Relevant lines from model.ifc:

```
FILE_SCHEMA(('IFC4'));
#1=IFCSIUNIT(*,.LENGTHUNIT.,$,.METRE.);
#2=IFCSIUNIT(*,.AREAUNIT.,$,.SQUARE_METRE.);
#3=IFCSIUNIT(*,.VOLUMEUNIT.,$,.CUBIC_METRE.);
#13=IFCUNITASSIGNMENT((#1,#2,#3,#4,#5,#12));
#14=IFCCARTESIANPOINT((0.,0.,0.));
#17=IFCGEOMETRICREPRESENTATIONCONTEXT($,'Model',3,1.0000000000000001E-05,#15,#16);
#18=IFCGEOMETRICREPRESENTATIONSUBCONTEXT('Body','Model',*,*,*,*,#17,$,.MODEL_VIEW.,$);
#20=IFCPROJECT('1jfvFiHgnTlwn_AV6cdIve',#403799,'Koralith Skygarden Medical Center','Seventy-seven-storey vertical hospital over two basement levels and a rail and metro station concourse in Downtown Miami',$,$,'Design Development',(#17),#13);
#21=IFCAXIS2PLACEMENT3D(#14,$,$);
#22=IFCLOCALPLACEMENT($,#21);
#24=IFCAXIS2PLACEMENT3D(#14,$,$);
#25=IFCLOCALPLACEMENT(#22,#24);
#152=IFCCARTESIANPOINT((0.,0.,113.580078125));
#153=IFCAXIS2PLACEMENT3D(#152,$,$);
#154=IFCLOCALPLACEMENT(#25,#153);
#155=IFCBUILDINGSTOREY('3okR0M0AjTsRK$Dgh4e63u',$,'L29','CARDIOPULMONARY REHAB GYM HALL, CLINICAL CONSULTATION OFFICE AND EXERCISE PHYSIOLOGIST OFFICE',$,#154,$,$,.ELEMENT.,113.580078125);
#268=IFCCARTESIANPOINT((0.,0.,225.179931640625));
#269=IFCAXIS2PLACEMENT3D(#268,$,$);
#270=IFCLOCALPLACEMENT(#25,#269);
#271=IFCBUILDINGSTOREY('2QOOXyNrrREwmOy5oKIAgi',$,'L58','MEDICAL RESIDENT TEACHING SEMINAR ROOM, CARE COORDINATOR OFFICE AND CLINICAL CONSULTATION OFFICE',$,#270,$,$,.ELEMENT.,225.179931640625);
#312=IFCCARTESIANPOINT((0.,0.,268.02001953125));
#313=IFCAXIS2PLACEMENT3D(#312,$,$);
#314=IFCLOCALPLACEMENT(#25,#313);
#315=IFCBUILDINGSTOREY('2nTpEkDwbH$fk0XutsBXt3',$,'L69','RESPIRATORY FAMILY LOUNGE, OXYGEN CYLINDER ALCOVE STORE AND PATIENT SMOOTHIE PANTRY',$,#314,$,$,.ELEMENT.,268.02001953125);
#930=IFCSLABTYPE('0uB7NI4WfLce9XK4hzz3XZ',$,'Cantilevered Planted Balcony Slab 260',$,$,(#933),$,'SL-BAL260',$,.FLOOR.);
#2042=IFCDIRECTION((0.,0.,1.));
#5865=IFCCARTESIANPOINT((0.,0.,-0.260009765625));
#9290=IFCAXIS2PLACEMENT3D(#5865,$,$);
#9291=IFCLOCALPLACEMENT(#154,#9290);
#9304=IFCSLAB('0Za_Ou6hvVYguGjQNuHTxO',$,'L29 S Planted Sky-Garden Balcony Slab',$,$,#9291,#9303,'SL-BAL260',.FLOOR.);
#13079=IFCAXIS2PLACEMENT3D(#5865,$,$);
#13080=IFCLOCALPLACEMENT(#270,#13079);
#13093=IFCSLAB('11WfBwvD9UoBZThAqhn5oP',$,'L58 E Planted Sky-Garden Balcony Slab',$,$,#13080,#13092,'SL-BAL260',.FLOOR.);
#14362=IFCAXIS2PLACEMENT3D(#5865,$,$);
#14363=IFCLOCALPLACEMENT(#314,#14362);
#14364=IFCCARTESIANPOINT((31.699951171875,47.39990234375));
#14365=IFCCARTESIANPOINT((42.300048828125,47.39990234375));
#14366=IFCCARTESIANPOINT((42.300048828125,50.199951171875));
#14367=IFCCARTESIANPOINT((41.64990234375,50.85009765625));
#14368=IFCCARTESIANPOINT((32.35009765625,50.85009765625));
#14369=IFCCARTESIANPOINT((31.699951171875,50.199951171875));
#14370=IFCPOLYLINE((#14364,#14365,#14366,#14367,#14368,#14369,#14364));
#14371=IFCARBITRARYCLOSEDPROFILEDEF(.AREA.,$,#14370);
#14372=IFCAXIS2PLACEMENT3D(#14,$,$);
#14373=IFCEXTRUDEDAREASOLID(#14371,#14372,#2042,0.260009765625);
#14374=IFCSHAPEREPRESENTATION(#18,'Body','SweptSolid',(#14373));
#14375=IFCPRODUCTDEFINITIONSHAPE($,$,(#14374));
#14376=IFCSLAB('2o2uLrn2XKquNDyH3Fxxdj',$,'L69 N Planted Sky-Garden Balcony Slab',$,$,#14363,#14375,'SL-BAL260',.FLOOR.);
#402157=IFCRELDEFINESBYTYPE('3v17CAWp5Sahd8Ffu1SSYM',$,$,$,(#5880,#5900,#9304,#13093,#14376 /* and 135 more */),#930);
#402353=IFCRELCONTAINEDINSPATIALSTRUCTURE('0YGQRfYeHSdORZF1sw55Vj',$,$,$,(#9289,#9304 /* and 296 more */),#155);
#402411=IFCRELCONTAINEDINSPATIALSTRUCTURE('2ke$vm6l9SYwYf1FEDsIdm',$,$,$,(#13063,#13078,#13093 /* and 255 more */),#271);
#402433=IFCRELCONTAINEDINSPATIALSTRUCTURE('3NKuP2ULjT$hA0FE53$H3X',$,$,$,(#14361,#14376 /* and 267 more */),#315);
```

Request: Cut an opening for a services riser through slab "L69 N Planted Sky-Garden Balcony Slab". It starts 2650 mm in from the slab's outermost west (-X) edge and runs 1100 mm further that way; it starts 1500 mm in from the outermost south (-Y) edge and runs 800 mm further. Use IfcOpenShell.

```python
import numpy as np
import ifcopenshell
import ifcopenshell.api.feature
import ifcopenshell.api.geometry
import ifcopenshell.api.root
import ifcopenshell.geom
import ifcopenshell.util.placement
import ifcopenshell.util.representation
import ifcopenshell.util.shape
import ifcopenshell.util.unit

model = ifcopenshell.open("model.ifc")
unit_scale = ifcopenshell.util.unit.calculate_unit_scale(model)
settings = ifcopenshell.geom.settings()


def volume(element):
    """Net volume in cubic metres, openings subtracted."""
    shape = ifcopenshell.geom.create_shape(settings, element)
    return ifcopenshell.util.shape.get_volume(shape.geometry)


slab = model.by_guid("2o2uLrn2XKquNDyH3Fxxdj")
before = volume(slab)

# Extent in the slab's own axes, in metres. The edges named are its -X and -Y sides.
slab_shape = ifcopenshell.geom.create_shape(settings, slab)
vertices = ifcopenshell.util.shape.get_vertices(slab_shape.geometry)
x_min, y_min, bottom = vertices.min(axis=0)
top = vertices[:, 2].max()

opening = ifcopenshell.api.root.create_entity(model, ifc_class="IfcOpeningElement", name="Services riser opening", predefined_type="OPENING")
context = ifcopenshell.util.representation.get_context(model, "Model", "Body", "MODEL_VIEW")
width, depth = 1.1, 0.8
outline = [(0.0, 0.0), (width, 0.0), (width, depth), (0.0, depth), (0.0, 0.0)]
# Overshoot both faces by 50 mm so the cut is clean.
shape = ifcopenshell.api.geometry.add_slab_representation(
    model, context=context, depth=top - bottom + 0.1, polyline=outline
)
ifcopenshell.api.geometry.assign_representation(model, product=opening, representation=shape)

matrix = ifcopenshell.util.placement.get_local_placement(slab.ObjectPlacement)
matrix[:, 3] = matrix @ np.append(np.array([x_min + 2.65, y_min + 1.5, bottom - 0.05]) / unit_scale, 1.0)
ifcopenshell.api.geometry.edit_object_placement(model, product=opening, matrix=matrix, is_si=False)
ifcopenshell.api.feature.add_feature(model, feature=opening, element=slab)

after = volume(slab)

print(f"slab volume {before:.3f} -> {after:.3f} m3")

model.write("model_rev.ifc")
```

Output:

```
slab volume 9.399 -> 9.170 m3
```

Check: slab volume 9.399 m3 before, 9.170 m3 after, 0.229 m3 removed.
